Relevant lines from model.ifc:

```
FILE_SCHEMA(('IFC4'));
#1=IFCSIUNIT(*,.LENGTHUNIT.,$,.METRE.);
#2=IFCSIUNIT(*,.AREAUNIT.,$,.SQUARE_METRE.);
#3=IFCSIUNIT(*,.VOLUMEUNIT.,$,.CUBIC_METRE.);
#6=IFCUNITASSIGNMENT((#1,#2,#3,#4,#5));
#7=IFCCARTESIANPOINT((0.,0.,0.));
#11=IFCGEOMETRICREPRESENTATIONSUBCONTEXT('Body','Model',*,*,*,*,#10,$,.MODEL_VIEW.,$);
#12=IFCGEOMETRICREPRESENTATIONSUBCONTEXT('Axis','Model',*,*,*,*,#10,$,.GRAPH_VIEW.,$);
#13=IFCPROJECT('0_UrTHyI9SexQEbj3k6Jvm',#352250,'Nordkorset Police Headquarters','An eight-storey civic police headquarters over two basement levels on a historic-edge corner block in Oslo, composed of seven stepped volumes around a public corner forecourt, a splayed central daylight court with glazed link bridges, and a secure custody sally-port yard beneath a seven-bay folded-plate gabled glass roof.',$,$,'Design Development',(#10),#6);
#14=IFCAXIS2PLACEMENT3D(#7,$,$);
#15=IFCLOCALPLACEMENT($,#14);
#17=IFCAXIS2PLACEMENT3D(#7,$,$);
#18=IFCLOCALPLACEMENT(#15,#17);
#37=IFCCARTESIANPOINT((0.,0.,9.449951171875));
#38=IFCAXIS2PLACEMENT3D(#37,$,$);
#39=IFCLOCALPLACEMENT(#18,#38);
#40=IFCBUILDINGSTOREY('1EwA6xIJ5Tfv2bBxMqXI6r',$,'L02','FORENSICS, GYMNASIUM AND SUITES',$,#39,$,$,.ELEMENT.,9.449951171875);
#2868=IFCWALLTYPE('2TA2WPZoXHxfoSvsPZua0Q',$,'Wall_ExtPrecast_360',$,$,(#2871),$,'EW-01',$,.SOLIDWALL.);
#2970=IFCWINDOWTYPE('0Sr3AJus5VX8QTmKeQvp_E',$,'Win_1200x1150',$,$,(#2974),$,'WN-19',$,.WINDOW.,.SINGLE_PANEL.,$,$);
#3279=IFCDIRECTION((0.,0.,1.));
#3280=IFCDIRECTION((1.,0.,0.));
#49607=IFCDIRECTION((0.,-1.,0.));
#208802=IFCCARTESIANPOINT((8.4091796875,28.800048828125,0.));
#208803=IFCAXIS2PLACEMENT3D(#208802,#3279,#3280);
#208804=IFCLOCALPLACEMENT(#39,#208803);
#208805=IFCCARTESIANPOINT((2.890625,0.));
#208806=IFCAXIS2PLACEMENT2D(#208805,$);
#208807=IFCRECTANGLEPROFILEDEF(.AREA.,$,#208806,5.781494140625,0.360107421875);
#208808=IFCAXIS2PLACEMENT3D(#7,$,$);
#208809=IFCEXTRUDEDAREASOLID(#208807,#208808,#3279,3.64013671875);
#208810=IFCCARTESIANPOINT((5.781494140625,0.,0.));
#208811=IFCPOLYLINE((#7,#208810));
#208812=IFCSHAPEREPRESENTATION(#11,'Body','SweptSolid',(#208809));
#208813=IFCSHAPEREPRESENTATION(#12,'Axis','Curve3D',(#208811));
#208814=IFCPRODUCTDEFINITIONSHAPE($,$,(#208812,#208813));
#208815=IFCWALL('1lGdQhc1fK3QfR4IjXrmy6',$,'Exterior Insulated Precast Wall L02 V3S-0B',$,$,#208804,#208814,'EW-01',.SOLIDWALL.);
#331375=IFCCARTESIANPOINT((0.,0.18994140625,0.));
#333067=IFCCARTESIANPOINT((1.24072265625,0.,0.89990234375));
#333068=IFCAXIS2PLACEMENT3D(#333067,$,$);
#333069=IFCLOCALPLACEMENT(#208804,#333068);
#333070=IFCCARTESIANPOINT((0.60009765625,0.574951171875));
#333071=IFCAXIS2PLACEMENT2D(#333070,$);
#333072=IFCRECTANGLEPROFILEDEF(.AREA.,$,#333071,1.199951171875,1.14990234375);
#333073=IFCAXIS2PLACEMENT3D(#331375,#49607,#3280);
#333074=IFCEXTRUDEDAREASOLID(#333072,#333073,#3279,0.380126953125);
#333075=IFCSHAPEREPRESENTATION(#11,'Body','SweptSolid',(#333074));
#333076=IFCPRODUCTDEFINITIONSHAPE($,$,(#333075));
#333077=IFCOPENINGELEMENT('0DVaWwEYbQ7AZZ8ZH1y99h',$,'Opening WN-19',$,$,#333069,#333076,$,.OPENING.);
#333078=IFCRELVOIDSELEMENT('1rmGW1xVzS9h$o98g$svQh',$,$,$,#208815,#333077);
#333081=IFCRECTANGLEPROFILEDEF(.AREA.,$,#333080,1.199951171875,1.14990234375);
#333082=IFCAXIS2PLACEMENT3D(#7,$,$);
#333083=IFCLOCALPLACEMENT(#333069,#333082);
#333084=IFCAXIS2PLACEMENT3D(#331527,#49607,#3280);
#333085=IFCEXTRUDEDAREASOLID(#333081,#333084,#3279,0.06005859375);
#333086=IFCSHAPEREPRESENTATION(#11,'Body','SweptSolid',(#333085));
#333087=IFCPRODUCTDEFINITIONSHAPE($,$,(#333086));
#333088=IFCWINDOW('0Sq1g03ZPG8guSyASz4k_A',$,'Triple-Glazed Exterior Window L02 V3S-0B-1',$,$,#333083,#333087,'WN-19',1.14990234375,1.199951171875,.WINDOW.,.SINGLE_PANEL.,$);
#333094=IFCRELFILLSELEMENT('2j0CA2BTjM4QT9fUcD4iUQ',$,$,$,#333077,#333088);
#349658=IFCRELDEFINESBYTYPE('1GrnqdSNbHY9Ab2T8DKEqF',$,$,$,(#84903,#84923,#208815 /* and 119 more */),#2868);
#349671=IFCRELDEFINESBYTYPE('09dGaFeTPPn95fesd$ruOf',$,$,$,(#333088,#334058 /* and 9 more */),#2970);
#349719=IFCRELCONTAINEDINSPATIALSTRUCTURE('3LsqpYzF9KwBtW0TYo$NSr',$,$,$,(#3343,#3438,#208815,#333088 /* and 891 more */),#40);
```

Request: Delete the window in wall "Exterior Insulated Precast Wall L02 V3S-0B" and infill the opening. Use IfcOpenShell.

```python
import ifcopenshell
import ifcopenshell.api.feature
import ifcopenshell.api.root
import ifcopenshell.geom
import ifcopenshell.util.shape

model = ifcopenshell.open("model.ifc")
settings = ifcopenshell.geom.settings()


def volume(element):
    """Net volume in cubic metres, openings subtracted."""
    shape = ifcopenshell.geom.create_shape(settings, element)
    return ifcopenshell.util.shape.get_volume(shape.geometry)


window = model.by_guid("0Sq1g03ZPG8guSyASz4k_A")
opening = window.FillsVoids[0].RelatingOpeningElement
wall = opening.VoidsElements[0].RelatingBuildingElement
before = volume(wall)

ifcopenshell.api.root.remove_product(model, product=window)
ifcopenshell.api.feature.remove_feature(model, feature=opening)

after = volume(wall)

print(f"wall volume {before:.3f} -> {after:.3f} m3")

model.write("model-out.ifc")
```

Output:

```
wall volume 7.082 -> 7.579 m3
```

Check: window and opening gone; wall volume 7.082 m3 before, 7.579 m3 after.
